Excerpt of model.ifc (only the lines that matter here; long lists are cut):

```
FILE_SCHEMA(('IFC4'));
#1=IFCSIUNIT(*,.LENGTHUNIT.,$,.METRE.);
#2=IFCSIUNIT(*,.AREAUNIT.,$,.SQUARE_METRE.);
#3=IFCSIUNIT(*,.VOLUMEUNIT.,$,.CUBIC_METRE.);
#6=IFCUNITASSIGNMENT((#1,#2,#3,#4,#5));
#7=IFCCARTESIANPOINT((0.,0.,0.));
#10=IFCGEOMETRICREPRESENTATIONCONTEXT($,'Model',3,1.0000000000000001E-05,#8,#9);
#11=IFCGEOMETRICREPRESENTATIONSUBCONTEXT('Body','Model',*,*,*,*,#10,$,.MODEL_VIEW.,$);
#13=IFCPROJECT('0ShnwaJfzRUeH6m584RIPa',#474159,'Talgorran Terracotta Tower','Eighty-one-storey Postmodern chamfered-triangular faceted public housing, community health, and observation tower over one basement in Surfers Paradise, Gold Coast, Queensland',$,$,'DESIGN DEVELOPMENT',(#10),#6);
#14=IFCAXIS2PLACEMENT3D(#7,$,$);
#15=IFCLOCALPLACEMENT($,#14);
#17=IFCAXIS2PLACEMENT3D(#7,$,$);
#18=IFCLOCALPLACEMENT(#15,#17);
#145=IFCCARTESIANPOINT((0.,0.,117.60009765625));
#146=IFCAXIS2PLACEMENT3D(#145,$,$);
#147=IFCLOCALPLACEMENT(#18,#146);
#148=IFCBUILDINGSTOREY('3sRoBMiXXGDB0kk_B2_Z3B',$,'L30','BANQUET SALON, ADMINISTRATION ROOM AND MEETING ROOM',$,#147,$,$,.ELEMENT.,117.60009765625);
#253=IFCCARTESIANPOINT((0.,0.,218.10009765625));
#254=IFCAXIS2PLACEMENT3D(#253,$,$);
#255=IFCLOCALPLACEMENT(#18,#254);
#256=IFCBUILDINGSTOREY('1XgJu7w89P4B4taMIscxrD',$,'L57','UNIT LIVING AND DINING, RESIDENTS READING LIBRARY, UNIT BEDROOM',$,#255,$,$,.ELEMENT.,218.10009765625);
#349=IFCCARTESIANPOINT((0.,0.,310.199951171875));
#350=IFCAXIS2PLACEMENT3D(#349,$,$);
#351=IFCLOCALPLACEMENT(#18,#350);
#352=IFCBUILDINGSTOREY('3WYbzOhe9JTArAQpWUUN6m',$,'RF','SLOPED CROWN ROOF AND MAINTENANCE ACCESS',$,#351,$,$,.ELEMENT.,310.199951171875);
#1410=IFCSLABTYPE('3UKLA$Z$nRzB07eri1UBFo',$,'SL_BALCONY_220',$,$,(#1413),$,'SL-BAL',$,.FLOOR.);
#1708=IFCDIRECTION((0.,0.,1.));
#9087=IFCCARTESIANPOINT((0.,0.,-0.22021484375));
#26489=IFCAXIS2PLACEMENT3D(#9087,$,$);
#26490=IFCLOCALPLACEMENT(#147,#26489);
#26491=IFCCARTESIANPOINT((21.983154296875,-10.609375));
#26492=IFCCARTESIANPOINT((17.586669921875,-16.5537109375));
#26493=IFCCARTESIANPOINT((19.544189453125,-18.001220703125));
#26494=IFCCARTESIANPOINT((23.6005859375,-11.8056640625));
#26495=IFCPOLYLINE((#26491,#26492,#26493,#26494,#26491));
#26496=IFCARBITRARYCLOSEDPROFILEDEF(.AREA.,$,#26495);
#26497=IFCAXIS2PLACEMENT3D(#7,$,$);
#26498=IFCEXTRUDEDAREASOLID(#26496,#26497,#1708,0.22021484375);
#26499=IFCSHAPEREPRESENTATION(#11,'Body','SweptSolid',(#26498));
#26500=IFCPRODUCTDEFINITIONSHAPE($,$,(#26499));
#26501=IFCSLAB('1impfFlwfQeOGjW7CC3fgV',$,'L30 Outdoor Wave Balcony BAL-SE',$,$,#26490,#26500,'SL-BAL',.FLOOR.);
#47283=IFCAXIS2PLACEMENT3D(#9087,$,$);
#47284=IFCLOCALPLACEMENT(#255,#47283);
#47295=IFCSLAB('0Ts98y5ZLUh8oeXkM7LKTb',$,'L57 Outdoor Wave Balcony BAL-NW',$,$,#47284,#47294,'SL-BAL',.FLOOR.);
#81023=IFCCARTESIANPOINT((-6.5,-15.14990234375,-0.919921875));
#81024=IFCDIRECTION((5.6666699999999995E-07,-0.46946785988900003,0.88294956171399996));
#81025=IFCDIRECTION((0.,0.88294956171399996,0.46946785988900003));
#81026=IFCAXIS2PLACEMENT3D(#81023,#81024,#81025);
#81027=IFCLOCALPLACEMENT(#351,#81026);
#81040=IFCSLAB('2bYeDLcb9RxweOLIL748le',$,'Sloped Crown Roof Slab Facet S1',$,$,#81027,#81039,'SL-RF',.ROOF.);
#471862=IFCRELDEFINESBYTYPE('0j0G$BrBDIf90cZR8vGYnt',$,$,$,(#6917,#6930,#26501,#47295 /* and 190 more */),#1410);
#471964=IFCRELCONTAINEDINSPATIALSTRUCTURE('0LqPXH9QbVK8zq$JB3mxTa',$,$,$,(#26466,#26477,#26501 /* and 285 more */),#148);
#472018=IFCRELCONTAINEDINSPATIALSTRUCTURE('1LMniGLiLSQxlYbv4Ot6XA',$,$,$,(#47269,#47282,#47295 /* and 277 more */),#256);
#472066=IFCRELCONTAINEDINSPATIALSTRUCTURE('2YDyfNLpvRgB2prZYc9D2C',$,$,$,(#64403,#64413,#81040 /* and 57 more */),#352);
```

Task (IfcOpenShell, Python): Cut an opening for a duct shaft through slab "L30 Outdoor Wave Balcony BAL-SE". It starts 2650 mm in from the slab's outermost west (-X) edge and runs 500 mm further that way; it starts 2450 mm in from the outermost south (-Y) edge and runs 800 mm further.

```python
import numpy as np
import ifcopenshell
import ifcopenshell.api.feature
import ifcopenshell.api.geometry
import ifcopenshell.api.root
import ifcopenshell.geom
import ifcopenshell.util.placement
import ifcopenshell.util.representation
import ifcopenshell.util.shape
import ifcopenshell.util.unit

model = ifcopenshell.open("model.ifc")
unit_scale = ifcopenshell.util.unit.calculate_unit_scale(model)
settings = ifcopenshell.geom.settings()


def volume(element):
    """Net volume in cubic metres, openings subtracted."""
    shape = ifcopenshell.geom.create_shape(settings, element)
    return ifcopenshell.util.shape.get_volume(shape.geometry)


slab = model.by_id(26501)
before = volume(slab)

# Extent in the slab's own axes, in metres. The edges named are its -X and -Y sides.
slab_shape = ifcopenshell.geom.create_shape(settings, slab)
vertices = ifcopenshell.util.shape.get_vertices(slab_shape.geometry)
x_min, y_min, bottom = vertices.min(axis=0)
top = vertices[:, 2].max()

opening = ifcopenshell.api.root.create_entity(model, ifc_class="IfcOpeningElement", name="Duct shaft opening", predefined_type="OPENING")
context = ifcopenshell.util.representation.get_context(model, "Model", "Body", "MODEL_VIEW")
width, depth = 0.5, 0.8
outline = [(0.0, 0.0), (width, 0.0), (width, depth), (0.0, depth), (0.0, 0.0)]
# Overshoot both faces by 50 mm so the cut is clean.
shape = ifcopenshell.api.geometry.add_slab_representation(
    model, context=context, depth=top - bottom + 0.1, polyline=outline
)
ifcopenshell.api.geometry.assign_representation(model, product=opening, representation=shape)

matrix = ifcopenshell.util.placement.get_local_placement(slab.ObjectPlacement)
matrix[:, 3] = matrix @ np.append(np.array([x_min + 2.65, y_min + 2.45, bottom - 0.05]) / unit_scale, 1.0)
ifcopenshell.api.geometry.edit_object_placement(model, product=opening, matrix=matrix, is_si=False)
ifcopenshell.api.feature.add_feature(model, feature=opening, element=slab)

after = volume(slab)

print(f"slab volume {before:.3f} -> {after:.3f} m3")

model.write("model-out.ifc")
```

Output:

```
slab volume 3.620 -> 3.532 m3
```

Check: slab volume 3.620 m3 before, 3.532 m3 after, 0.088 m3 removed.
